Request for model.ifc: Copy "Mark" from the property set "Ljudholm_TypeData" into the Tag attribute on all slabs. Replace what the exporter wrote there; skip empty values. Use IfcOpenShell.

First a look at what the model holds.

```python
import ifcopenshell
import ifcopenshell.util.element

model = ifcopenshell.open("model.ifc")
print(model.schema)
slabs = model.by_type("IfcSlab")
print(len(slabs), "slabs")
for e in slabs[:8]:
    source = ifcopenshell.util.element.get_pset(e, "Ljudholm_TypeData", "Mark")
    target = e.Tag
    print(e.id(), repr(source), repr(target), sep=" | ")
```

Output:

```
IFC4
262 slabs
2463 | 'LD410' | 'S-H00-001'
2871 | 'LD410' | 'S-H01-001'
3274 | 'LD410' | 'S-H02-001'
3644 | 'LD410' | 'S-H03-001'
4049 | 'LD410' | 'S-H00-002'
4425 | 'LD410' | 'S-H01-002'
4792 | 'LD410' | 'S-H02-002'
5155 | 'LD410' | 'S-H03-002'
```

```python
import ifcopenshell
import ifcopenshell.util.element

model = ifcopenshell.open("model.ifc")

count = 0
for e in model.by_type("IfcSlab"):
    value = ifcopenshell.util.element.get_pset(e, "Ljudholm_TypeData", "Mark")
    current = e.Tag
    if not value or not value.strip() or current == value:
        continue
    e.Tag = value
    count += 1

print(count, "slabs updated")

model.write("model_edited.ifc")
```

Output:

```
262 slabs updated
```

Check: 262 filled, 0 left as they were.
